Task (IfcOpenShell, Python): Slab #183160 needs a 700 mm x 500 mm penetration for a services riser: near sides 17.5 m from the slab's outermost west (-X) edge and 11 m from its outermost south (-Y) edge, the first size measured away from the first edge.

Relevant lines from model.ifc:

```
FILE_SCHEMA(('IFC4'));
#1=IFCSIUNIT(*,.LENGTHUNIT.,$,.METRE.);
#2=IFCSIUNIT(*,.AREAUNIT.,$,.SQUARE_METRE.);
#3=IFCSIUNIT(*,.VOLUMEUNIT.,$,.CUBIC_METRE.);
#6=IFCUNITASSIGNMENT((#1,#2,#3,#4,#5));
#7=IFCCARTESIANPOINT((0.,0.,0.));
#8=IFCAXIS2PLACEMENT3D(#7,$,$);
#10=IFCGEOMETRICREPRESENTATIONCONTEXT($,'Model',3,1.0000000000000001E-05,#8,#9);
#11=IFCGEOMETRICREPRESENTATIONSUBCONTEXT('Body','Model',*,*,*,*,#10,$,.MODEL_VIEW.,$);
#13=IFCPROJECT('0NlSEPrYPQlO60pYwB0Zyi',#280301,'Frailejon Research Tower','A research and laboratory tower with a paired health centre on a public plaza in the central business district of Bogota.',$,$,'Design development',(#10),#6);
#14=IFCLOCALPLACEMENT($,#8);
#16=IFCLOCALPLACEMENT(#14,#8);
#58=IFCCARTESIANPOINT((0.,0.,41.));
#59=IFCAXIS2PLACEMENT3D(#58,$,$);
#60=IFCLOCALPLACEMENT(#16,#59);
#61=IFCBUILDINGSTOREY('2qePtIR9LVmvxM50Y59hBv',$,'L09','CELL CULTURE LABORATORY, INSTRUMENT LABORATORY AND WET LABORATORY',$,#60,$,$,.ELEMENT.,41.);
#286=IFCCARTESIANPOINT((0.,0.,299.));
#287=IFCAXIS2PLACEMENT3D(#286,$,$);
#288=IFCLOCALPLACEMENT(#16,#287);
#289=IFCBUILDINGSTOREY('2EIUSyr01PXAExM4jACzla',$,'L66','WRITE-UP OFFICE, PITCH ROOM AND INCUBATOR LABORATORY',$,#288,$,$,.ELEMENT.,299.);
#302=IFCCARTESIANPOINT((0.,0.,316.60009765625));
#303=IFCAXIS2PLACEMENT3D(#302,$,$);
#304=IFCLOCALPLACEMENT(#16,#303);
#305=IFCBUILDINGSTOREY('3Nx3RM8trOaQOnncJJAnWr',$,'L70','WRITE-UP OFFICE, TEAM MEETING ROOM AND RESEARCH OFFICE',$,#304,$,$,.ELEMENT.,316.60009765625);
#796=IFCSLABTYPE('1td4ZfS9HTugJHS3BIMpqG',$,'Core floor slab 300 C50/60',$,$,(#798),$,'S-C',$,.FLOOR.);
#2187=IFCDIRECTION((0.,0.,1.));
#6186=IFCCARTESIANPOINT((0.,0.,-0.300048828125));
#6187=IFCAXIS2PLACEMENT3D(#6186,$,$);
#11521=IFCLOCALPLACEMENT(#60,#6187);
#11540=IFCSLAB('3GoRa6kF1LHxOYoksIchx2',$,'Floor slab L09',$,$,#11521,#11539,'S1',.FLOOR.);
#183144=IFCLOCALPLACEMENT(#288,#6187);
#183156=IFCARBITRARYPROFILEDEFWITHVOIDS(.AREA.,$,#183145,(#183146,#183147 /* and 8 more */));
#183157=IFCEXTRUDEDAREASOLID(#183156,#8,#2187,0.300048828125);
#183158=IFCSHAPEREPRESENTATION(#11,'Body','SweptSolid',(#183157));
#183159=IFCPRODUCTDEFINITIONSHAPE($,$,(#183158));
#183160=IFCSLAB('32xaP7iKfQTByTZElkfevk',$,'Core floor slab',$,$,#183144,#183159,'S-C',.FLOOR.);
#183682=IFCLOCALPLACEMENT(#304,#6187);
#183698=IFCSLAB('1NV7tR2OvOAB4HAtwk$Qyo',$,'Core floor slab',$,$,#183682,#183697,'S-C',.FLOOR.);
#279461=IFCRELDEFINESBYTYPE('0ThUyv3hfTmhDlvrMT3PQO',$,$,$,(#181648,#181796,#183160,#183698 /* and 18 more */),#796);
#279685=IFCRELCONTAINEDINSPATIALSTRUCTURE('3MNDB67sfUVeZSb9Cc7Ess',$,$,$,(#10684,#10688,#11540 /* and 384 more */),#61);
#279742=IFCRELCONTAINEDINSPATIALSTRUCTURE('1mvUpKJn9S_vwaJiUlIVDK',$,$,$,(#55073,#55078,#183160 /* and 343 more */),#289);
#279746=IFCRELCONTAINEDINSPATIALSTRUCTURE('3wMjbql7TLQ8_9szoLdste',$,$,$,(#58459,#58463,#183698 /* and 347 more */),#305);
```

```python
import numpy as np
import ifcopenshell
import ifcopenshell.api.feature
import ifcopenshell.api.geometry
import ifcopenshell.api.root
import ifcopenshell.geom
import ifcopenshell.util.placement
import ifcopenshell.util.representation
import ifcopenshell.util.shape
import ifcopenshell.util.unit

model = ifcopenshell.open("model.ifc")
unit_scale = ifcopenshell.util.unit.calculate_unit_scale(model)
settings = ifcopenshell.geom.settings()


def volume(element):
    """Net volume in cubic metres, openings subtracted."""
    shape = ifcopenshell.geom.create_shape(settings, element)
    return ifcopenshell.util.shape.get_volume(shape.geometry)


slab = model.by_guid("32xaP7iKfQTByTZElkfevk")
before = volume(slab)

# Extent in the slab's own axes, in metres. The edges named are its -X and -Y sides.
slab_shape = ifcopenshell.geom.create_shape(settings, slab)
vertices = ifcopenshell.util.shape.get_vertices(slab_shape.geometry)
x_min, y_min, bottom = vertices.min(axis=0)
top = vertices[:, 2].max()

opening = ifcopenshell.api.root.create_entity(model, ifc_class="IfcOpeningElement", name="Services riser opening", predefined_type="OPENING")
context = ifcopenshell.util.representation.get_context(model, "Model", "Body", "MODEL_VIEW")
width, depth = 0.7, 0.5
outline = [(0.0, 0.0), (width, 0.0), (width, depth), (0.0, depth), (0.0, 0.0)]
# Overshoot both faces by 50 mm so the cut is clean.
shape = ifcopenshell.api.geometry.add_slab_representation(
    model, context=context, depth=top - bottom + 0.1, polyline=outline
)
ifcopenshell.api.geometry.assign_representation(model, product=opening, representation=shape)

matrix = ifcopenshell.util.placement.get_local_placement(slab.ObjectPlacement)
matrix[:, 3] = matrix @ np.append(np.array([x_min + 17.5, y_min + 11, bottom - 0.05]) / unit_scale, 1.0)
ifcopenshell.api.geometry.edit_object_placement(model, product=opening, matrix=matrix, is_si=False)
ifcopenshell.api.feature.add_feature(model, feature=opening, element=slab)

after = volume(slab)

print(f"slab volume {before:.3f} -> {after:.3f} m3")

model.write("model_edited.ifc")
```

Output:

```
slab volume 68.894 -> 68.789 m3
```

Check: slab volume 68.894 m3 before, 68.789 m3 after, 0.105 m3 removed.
